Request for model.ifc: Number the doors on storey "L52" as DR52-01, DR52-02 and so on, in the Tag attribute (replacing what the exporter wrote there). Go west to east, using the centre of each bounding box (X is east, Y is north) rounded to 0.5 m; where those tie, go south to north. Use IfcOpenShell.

First a look at what the model holds.

```python
import ifcopenshell
import ifcopenshell.util.element
import ifcopenshell.util.placement

model = ifcopenshell.open("model.ifc")
print(model.schema)
storey = next(s for s in model.by_type("IfcBuildingStorey") if s.Name == "L52")
doors = [e for e in ifcopenshell.util.element.get_decomposition(storey) if e.is_a("IfcDoor")]
for e in sorted(doors, key=lambda e: e.id()):
    origin = ifcopenshell.util.placement.get_local_placement(e.ObjectPlacement)[:3, 3]
    print(e.id(), e.Tag, e.Name, origin.round(2) + 0.0, sep=" | ")
```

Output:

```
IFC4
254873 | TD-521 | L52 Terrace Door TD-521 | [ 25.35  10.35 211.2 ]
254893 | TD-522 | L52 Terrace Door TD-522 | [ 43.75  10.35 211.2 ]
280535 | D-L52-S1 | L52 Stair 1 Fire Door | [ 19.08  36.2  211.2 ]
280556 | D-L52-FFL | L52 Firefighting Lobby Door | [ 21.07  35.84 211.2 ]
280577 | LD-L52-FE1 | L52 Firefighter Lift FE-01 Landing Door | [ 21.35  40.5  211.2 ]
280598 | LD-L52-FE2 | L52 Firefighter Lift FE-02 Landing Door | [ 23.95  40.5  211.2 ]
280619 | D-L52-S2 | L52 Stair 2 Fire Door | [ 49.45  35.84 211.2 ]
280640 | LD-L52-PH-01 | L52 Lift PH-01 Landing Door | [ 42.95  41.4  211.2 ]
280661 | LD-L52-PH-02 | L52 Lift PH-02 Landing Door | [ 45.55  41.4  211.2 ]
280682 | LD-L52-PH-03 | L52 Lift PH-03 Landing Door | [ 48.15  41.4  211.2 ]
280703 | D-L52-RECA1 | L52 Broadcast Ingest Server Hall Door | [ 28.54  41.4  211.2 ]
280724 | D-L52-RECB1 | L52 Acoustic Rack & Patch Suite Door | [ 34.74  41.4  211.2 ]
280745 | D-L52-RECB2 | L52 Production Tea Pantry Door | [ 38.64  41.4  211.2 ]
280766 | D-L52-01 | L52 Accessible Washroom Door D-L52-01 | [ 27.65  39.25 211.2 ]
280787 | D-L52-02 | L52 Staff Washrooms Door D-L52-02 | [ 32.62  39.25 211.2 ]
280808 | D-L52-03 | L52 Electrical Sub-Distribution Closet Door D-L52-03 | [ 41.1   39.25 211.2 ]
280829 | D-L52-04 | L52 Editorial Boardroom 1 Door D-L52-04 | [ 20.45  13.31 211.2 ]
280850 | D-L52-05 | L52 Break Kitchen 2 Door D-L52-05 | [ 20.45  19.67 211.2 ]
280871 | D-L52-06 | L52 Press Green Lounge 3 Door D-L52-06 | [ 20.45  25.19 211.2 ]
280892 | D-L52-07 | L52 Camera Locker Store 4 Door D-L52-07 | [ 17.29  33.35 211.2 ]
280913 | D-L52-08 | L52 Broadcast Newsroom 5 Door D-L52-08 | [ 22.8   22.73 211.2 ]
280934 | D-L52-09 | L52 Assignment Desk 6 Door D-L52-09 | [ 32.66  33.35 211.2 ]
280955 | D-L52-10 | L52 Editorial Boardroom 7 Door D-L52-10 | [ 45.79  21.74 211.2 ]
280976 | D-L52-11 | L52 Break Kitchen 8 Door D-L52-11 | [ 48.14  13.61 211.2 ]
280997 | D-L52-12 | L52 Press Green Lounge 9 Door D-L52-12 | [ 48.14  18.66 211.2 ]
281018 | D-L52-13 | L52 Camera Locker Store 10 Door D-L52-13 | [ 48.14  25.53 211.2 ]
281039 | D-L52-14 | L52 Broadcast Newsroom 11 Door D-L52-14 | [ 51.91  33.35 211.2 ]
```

```python
import ifcopenshell
import ifcopenshell.geom
import ifcopenshell.util.element
import ifcopenshell.util.shape

model = ifcopenshell.open("model.ifc")
settings = ifcopenshell.geom.settings()
settings.set("use-world-coords", True)


def centre(element):
    shape = ifcopenshell.geom.create_shape(settings, element)
    return ifcopenshell.util.shape.get_bbox_centroid(shape.geometry)


storey = next(s for s in model.by_type("IfcBuildingStorey") if s.Name == "L52")
doors = [e for e in ifcopenshell.util.element.get_decomposition(storey) if e.is_a("IfcDoor")]

# Insertion points can sit at a corner or the storey origin, so sort by the geometry (in metres).
centres = {e: centre(e) for e in doors}
doors.sort(key=lambda e: (round(centres[e][0] / 0.5), centres[e][1]))

for i, e in enumerate(doors, start=1):
    number = f"DR52-{i:02d}"
    e.Tag = number
    print(e.id(), number)

model.write("model-out.ifc")
```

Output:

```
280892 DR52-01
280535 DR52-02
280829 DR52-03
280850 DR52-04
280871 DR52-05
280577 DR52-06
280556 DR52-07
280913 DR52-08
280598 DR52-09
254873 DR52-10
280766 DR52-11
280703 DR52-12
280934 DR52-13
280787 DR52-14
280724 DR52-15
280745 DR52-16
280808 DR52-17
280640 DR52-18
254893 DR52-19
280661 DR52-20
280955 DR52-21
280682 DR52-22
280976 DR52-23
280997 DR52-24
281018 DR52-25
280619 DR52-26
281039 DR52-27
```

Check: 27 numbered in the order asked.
